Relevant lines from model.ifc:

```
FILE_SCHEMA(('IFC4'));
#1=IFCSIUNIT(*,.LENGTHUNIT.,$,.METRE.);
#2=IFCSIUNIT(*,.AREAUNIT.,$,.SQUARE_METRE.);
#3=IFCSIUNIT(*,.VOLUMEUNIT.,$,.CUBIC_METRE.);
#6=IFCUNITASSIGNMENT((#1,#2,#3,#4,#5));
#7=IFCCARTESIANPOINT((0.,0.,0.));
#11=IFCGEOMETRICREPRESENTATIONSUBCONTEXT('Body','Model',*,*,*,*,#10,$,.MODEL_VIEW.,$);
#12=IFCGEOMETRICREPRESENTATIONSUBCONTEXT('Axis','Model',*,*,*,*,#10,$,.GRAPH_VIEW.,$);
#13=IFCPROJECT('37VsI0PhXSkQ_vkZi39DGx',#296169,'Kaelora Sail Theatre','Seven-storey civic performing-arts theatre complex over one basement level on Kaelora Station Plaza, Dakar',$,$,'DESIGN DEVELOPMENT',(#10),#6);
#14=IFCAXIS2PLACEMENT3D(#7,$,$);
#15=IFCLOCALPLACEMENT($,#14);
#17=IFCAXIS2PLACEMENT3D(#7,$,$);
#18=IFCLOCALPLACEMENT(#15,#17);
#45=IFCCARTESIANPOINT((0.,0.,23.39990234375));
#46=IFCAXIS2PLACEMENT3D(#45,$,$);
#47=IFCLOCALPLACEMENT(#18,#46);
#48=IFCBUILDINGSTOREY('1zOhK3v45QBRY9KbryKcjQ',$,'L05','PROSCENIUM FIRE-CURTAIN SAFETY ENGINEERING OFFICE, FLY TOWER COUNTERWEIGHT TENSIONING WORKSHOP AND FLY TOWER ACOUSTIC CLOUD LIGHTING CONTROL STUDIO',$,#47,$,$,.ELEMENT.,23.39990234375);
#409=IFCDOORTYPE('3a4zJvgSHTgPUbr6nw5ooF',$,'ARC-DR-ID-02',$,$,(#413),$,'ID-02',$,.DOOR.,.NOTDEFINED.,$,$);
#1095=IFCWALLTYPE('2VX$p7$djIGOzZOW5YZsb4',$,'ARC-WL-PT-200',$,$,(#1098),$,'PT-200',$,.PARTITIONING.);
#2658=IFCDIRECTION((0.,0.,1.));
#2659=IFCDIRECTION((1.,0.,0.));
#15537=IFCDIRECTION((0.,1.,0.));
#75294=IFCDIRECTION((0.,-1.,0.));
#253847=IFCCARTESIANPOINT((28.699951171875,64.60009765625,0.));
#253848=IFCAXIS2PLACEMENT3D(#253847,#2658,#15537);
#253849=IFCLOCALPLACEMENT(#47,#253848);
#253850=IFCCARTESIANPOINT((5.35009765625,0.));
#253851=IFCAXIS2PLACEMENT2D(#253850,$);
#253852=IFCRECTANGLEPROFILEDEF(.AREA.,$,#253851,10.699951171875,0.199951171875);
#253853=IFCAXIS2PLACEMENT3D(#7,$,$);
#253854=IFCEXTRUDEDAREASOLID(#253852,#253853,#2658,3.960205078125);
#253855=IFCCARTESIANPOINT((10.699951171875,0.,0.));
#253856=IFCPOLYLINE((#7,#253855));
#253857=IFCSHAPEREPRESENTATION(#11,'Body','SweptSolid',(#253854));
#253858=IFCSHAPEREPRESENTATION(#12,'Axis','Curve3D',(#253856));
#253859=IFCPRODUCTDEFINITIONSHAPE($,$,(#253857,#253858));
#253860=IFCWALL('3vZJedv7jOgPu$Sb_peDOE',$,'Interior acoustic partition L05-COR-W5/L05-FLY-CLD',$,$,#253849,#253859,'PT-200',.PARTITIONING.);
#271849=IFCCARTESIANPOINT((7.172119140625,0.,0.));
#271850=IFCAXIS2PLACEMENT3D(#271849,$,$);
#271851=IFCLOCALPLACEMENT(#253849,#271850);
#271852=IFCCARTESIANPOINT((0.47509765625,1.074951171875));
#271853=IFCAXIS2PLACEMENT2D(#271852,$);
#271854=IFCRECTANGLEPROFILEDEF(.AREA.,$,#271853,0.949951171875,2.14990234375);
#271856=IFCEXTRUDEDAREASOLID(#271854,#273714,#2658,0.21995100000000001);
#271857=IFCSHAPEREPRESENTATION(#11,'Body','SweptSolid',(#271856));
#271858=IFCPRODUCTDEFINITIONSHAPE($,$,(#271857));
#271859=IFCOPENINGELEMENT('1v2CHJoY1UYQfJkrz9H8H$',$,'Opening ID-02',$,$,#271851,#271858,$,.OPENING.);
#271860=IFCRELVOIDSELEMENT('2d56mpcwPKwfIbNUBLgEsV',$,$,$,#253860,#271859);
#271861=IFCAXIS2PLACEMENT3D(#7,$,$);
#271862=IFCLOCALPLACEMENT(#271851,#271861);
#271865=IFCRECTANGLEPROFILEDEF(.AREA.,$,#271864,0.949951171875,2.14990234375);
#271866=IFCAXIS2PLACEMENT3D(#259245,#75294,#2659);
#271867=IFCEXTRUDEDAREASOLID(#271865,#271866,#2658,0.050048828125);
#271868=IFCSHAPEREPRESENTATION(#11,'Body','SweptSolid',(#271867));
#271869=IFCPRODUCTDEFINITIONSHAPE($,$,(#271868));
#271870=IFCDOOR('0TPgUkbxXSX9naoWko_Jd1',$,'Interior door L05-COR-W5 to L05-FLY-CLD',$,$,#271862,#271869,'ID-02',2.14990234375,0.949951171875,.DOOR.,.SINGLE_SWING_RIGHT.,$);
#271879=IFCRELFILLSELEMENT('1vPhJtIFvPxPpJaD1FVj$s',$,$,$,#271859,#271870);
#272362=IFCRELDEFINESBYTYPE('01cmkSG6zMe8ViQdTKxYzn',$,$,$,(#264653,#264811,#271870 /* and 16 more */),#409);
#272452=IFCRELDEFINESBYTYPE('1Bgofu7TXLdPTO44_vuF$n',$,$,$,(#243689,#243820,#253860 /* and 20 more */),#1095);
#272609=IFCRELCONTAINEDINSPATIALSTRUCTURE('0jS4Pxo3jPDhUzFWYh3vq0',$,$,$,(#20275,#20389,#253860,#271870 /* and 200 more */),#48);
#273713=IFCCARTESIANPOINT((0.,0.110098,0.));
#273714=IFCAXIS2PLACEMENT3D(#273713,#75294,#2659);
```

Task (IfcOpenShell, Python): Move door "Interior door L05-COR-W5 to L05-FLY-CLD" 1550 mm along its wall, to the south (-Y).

```python
import ifcopenshell
import ifcopenshell.api.geometry
import ifcopenshell.util.placement

model = ifcopenshell.open("model.ifc")

door = model.by_guid("0TPgUkbxXSX9naoWko_Jd1")
opening = door.FillsVoids[0].RelatingOpeningElement
wall = opening.VoidsElements[0].RelatingBuildingElement

wall_matrix = ifcopenshell.util.placement.get_local_placement(wall.ObjectPlacement)
shift = wall_matrix[:3, 0] * -1.55
before = ifcopenshell.util.placement.get_local_placement(door.ObjectPlacement)[:3, 3].copy()

# The door is placed relative to its opening, so it follows when the opening moves.
matrix = ifcopenshell.util.placement.get_local_placement(opening.ObjectPlacement)
matrix[:3, 3] += shift
ifcopenshell.api.geometry.edit_object_placement(
    model, product=opening, matrix=matrix, is_si=False, should_transform_children=True
)

after = ifcopenshell.util.placement.get_local_placement(door.ObjectPlacement)[:3, 3]
print("door moved by", (after - before).round(3) + 0.0)

model.write("model_rev.ifc")
```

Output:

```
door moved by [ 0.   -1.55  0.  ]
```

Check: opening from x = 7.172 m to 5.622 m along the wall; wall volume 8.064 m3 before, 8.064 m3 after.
